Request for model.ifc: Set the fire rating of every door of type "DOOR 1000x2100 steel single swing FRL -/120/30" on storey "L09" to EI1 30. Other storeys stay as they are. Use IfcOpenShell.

First a look at what the model holds.

```python
import ifcopenshell
import ifcopenshell.util.element

model = ifcopenshell.open("model.ifc")
print(model.schema)
storey = next(s for s in model.by_type("IfcBuildingStorey") if s.Name == "L09")
doors = [e for e in ifcopenshell.util.element.get_decomposition(storey) if e.is_a("IfcDoor")]
seen = {}
for e in doors:
    element_type = ifcopenshell.util.element.get_type(e)
    key = (element_type.Name if element_type != e and element_type else None, ifcopenshell.util.element.get_pset(e, "Pset_DoorCommon", "FireRating"))
    seen[key] = seen.get(key, 0) + 1
for (name, value), count in sorted(seen.items(), key=str):
    print(count, "x", name, "|", value)
```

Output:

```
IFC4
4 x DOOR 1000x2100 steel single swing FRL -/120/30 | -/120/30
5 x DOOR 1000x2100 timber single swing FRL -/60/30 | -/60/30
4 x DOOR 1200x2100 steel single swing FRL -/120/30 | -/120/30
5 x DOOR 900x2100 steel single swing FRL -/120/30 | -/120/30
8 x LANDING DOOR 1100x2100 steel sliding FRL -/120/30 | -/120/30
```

```python
import ifcopenshell
import ifcopenshell.api.pset
import ifcopenshell.util.element

model = ifcopenshell.open("model.ifc")

storey = next(s for s in model.by_type("IfcBuildingStorey") if s.Name == "L09")
doors = [e for e in ifcopenshell.util.element.get_decomposition(storey) if e.is_a("IfcDoor")]

count = 0
for e in doors:
    element_type = ifcopenshell.util.element.get_type(e)
    if element_type in (None, e) or element_type.Name != "DOOR 1000x2100 steel single swing FRL -/120/30":
        continue
    # add_pset returns the element's existing set when there is one.
    pset = ifcopenshell.api.pset.add_pset(model, product=e, name="Pset_DoorCommon")
    ifcopenshell.api.pset.edit_pset(model, pset=pset, properties={"FireRating": "EI1 30"})
    count += 1

print(count, "doors updated")

model.write("model_updated.ifc")
```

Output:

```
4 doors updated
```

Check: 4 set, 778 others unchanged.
